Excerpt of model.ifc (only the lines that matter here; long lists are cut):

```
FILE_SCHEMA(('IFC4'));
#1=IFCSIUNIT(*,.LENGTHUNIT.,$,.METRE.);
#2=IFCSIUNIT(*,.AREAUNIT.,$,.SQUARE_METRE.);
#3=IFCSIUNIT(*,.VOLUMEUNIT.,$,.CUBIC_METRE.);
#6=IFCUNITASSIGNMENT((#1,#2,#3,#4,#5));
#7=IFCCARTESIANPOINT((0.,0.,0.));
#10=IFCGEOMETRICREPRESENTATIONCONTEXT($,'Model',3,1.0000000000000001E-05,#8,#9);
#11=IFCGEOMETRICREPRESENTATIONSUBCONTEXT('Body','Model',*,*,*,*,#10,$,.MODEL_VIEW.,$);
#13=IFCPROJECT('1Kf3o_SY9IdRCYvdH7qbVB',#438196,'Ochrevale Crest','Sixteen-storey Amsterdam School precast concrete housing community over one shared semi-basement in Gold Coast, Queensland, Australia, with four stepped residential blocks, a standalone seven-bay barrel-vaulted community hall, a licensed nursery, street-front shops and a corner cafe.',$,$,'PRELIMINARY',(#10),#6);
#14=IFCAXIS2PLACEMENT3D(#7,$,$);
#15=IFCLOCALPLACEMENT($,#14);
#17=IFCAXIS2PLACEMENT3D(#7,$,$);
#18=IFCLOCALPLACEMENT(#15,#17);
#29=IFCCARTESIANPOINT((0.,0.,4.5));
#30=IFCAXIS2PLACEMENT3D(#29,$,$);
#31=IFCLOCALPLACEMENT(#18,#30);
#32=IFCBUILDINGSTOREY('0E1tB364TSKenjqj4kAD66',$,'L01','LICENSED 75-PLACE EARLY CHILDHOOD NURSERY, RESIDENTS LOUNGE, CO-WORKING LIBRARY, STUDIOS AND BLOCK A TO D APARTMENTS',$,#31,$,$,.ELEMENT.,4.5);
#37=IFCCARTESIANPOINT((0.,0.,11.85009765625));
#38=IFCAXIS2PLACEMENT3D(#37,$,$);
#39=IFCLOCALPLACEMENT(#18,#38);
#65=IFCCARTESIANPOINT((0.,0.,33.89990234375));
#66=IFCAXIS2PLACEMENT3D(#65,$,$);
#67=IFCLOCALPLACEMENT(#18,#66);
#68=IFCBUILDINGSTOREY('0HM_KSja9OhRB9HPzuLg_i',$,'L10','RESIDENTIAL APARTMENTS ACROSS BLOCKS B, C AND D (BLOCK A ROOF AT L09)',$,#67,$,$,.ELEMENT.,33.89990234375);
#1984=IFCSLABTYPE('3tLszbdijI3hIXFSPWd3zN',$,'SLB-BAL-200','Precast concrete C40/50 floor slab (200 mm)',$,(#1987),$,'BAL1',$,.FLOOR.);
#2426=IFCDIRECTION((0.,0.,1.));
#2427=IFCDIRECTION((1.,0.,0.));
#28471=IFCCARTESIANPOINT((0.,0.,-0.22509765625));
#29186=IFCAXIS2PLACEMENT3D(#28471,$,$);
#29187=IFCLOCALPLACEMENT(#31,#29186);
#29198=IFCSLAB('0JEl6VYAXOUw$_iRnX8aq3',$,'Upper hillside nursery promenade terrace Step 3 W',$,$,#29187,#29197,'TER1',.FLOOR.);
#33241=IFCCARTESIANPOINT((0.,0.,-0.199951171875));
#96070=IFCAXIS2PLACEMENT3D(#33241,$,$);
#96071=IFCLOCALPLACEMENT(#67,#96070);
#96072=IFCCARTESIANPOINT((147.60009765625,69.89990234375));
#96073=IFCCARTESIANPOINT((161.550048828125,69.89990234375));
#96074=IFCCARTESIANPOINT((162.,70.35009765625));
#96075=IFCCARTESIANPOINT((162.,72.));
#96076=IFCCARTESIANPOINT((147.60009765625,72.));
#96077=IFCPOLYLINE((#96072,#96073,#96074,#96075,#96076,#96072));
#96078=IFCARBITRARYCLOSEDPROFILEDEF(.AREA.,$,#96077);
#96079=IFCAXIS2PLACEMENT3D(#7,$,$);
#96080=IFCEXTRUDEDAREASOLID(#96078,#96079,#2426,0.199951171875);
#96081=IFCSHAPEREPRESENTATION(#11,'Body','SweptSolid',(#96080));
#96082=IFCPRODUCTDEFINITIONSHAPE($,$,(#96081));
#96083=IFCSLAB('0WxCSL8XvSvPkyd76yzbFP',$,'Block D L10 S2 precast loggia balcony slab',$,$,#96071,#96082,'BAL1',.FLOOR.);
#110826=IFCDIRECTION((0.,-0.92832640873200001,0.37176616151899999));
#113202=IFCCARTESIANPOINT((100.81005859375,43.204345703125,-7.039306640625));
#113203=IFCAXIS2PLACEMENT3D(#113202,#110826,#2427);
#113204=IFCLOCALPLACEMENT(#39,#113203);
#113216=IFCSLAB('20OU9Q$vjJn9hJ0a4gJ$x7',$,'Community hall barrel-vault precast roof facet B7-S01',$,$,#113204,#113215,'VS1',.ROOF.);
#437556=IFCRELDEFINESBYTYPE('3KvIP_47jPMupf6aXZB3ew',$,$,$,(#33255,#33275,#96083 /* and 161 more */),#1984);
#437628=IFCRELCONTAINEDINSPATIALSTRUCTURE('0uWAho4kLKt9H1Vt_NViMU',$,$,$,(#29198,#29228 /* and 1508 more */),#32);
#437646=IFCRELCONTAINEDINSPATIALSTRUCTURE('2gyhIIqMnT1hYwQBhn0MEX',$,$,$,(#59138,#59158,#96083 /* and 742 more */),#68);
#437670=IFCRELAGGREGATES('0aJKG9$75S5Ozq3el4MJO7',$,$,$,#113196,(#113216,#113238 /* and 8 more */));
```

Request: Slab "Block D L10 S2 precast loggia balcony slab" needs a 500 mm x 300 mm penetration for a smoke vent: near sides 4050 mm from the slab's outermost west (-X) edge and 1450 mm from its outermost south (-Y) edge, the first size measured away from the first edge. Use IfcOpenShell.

```python
import numpy as np
import ifcopenshell
import ifcopenshell.api.feature
import ifcopenshell.api.geometry
import ifcopenshell.api.root
import ifcopenshell.geom
import ifcopenshell.util.placement
import ifcopenshell.util.representation
import ifcopenshell.util.shape
import ifcopenshell.util.unit

model = ifcopenshell.open("model.ifc")
unit_scale = ifcopenshell.util.unit.calculate_unit_scale(model)
settings = ifcopenshell.geom.settings()


def volume(element):
    """Net volume in cubic metres, openings subtracted."""
    shape = ifcopenshell.geom.create_shape(settings, element)
    return ifcopenshell.util.shape.get_volume(shape.geometry)


slab = model.by_guid("0WxCSL8XvSvPkyd76yzbFP")
before = volume(slab)

# Extent in the slab's own axes, in metres. The edges named are its -X and -Y sides.
slab_shape = ifcopenshell.geom.create_shape(settings, slab)
vertices = ifcopenshell.util.shape.get_vertices(slab_shape.geometry)
x_min, y_min, bottom = vertices.min(axis=0)
top = vertices[:, 2].max()

opening = ifcopenshell.api.root.create_entity(model, ifc_class="IfcOpeningElement", name="Smoke vent opening", predefined_type="OPENING")
context = ifcopenshell.util.representation.get_context(model, "Model", "Body", "MODEL_VIEW")
width, depth = 0.5, 0.3
outline = [(0.0, 0.0), (width, 0.0), (width, depth), (0.0, depth), (0.0, 0.0)]
# Overshoot both faces by 50 mm so the cut is clean.
shape = ifcopenshell.api.geometry.add_slab_representation(
    model, context=context, depth=top - bottom + 0.1, polyline=outline
)
ifcopenshell.api.geometry.assign_representation(model, product=opening, representation=shape)

matrix = ifcopenshell.util.placement.get_local_placement(slab.ObjectPlacement)
matrix[:, 3] = matrix @ np.append(np.array([x_min + 4.05, y_min + 1.45, bottom - 0.05]) / unit_scale, 1.0)
ifcopenshell.api.geometry.edit_object_placement(model, product=opening, matrix=matrix, is_si=False)
ifcopenshell.api.feature.add_feature(model, feature=opening, element=slab)

after = volume(slab)

print(f"slab volume {before:.3f} -> {after:.3f} m3")

model.write("model_rev.ifc")
```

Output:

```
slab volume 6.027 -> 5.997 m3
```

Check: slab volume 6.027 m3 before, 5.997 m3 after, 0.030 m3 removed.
